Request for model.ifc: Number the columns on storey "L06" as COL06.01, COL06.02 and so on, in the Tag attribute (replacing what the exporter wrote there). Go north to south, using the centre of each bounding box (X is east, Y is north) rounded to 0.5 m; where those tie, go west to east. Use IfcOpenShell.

First a look at what the model holds.

```python
import ifcopenshell
import ifcopenshell.util.element
import ifcopenshell.util.placement

model = ifcopenshell.open("model.ifc")
print(model.schema)
storey = next(s for s in model.by_type("IfcBuildingStorey") if s.Name == "L06")
columns = [e for e in ifcopenshell.util.element.get_decomposition(storey) if e.is_a("IfcColumn")]
for e in sorted(columns, key=lambda e: e.id()):
    origin = ifcopenshell.util.placement.get_local_placement(e.ObjectPlacement)[:3, 3]
    print(e.id(), e.Tag, e.Name, origin.round(2) + 0.0, sep=" | ")
```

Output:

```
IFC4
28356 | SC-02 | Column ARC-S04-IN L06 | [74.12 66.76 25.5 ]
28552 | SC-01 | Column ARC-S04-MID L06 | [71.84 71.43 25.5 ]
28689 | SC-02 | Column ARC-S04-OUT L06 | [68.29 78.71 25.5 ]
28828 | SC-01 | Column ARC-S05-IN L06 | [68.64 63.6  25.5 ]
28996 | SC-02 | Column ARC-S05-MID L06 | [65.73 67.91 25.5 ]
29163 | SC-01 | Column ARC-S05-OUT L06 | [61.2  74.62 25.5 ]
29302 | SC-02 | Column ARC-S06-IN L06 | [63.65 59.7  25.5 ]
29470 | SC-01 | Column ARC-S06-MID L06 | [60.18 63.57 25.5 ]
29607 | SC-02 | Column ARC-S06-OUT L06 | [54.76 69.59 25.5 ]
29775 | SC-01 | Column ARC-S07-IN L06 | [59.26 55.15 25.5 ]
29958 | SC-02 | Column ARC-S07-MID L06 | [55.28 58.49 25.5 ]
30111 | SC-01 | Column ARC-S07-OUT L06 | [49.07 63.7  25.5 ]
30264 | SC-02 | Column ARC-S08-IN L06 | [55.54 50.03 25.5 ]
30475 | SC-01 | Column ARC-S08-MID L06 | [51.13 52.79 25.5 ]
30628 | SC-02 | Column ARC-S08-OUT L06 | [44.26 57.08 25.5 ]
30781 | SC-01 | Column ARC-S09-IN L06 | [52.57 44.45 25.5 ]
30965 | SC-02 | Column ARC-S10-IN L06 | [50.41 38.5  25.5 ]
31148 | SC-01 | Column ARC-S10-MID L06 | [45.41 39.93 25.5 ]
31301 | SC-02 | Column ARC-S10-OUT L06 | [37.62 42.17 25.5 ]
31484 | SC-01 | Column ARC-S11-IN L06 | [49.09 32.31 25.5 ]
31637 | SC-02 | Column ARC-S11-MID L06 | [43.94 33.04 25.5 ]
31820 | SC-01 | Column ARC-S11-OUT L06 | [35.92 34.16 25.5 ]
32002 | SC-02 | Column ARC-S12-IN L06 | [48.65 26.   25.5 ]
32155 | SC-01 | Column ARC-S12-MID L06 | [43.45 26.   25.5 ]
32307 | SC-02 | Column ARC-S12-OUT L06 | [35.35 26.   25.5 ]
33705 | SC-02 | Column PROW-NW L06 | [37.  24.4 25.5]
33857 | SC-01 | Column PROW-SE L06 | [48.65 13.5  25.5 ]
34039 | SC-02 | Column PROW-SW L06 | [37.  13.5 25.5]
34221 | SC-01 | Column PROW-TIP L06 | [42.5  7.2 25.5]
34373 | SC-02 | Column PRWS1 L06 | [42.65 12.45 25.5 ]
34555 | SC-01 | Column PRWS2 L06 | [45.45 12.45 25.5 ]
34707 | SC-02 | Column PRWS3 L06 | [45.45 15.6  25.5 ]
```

```python
import ifcopenshell
import ifcopenshell.geom
import ifcopenshell.util.element
import ifcopenshell.util.shape

model = ifcopenshell.open("model.ifc")
settings = ifcopenshell.geom.settings()
settings.set("use-world-coords", True)


def centre(element):
    shape = ifcopenshell.geom.create_shape(settings, element)
    return ifcopenshell.util.shape.get_bbox_centroid(shape.geometry)


storey = next(s for s in model.by_type("IfcBuildingStorey") if s.Name == "L06")
columns = [e for e in ifcopenshell.util.element.get_decomposition(storey) if e.is_a("IfcColumn")]

# Insertion points can sit at a corner or the storey origin, so sort by the geometry (in metres).
centres = {e: centre(e) for e in columns}
columns.sort(key=lambda e: (-round(centres[e][1] / 0.5), centres[e][0]))

for i, e in enumerate(columns, start=1):
    number = f"COL06.{i:02d}"
    e.Tag = number
    print(e.id(), number)

model.write("model_rev.ifc")
```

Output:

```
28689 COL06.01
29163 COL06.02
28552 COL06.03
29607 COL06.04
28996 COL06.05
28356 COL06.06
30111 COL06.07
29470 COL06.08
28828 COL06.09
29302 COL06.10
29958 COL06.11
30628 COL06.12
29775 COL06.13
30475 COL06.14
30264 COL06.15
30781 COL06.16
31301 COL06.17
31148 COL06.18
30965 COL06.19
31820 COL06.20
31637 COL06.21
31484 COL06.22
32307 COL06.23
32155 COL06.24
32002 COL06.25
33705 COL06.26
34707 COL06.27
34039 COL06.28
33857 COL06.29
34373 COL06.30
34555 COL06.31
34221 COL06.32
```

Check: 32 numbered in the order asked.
